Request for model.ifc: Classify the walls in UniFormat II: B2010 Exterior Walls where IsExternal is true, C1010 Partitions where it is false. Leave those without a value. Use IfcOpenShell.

First a look at what the model holds.

```python
import ifcopenshell
import ifcopenshell.util.element

model = ifcopenshell.open("model.ifc")
print(model.schema)
print("classifications:", [c.Name for c in model.by_type("IfcClassification")])
values = [ifcopenshell.util.element.get_pset(e, "Pset_WallCommon", "IsExternal") for e in model.by_type("IfcWall")]
for value in (True, False, None):
    print("IsExternal", value, values.count(value))
```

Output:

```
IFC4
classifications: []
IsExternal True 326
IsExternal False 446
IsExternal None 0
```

```python
import ifcopenshell
import ifcopenshell.api.classification
import ifcopenshell.util.element

model = ifcopenshell.open("model.ifc")

system = ifcopenshell.api.classification.add_classification(model, classification="UniFormat II")

walls = model.by_type("IfcWall")
external = {e: ifcopenshell.util.element.get_pset(e, "Pset_WallCommon", "IsExternal") for e in walls}
for flag, code, name in ((True, "B2010", "Exterior Walls"), (False, "C1010", "Partitions")):
    products = [e for e in walls if external[e] is flag]
    ifcopenshell.api.classification.add_reference(
        model, products=products, classification=system, identification=code, name=name
    )
    print(code, len(products))

model.write("model_updated.ifc")
```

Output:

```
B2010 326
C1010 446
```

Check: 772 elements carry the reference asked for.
